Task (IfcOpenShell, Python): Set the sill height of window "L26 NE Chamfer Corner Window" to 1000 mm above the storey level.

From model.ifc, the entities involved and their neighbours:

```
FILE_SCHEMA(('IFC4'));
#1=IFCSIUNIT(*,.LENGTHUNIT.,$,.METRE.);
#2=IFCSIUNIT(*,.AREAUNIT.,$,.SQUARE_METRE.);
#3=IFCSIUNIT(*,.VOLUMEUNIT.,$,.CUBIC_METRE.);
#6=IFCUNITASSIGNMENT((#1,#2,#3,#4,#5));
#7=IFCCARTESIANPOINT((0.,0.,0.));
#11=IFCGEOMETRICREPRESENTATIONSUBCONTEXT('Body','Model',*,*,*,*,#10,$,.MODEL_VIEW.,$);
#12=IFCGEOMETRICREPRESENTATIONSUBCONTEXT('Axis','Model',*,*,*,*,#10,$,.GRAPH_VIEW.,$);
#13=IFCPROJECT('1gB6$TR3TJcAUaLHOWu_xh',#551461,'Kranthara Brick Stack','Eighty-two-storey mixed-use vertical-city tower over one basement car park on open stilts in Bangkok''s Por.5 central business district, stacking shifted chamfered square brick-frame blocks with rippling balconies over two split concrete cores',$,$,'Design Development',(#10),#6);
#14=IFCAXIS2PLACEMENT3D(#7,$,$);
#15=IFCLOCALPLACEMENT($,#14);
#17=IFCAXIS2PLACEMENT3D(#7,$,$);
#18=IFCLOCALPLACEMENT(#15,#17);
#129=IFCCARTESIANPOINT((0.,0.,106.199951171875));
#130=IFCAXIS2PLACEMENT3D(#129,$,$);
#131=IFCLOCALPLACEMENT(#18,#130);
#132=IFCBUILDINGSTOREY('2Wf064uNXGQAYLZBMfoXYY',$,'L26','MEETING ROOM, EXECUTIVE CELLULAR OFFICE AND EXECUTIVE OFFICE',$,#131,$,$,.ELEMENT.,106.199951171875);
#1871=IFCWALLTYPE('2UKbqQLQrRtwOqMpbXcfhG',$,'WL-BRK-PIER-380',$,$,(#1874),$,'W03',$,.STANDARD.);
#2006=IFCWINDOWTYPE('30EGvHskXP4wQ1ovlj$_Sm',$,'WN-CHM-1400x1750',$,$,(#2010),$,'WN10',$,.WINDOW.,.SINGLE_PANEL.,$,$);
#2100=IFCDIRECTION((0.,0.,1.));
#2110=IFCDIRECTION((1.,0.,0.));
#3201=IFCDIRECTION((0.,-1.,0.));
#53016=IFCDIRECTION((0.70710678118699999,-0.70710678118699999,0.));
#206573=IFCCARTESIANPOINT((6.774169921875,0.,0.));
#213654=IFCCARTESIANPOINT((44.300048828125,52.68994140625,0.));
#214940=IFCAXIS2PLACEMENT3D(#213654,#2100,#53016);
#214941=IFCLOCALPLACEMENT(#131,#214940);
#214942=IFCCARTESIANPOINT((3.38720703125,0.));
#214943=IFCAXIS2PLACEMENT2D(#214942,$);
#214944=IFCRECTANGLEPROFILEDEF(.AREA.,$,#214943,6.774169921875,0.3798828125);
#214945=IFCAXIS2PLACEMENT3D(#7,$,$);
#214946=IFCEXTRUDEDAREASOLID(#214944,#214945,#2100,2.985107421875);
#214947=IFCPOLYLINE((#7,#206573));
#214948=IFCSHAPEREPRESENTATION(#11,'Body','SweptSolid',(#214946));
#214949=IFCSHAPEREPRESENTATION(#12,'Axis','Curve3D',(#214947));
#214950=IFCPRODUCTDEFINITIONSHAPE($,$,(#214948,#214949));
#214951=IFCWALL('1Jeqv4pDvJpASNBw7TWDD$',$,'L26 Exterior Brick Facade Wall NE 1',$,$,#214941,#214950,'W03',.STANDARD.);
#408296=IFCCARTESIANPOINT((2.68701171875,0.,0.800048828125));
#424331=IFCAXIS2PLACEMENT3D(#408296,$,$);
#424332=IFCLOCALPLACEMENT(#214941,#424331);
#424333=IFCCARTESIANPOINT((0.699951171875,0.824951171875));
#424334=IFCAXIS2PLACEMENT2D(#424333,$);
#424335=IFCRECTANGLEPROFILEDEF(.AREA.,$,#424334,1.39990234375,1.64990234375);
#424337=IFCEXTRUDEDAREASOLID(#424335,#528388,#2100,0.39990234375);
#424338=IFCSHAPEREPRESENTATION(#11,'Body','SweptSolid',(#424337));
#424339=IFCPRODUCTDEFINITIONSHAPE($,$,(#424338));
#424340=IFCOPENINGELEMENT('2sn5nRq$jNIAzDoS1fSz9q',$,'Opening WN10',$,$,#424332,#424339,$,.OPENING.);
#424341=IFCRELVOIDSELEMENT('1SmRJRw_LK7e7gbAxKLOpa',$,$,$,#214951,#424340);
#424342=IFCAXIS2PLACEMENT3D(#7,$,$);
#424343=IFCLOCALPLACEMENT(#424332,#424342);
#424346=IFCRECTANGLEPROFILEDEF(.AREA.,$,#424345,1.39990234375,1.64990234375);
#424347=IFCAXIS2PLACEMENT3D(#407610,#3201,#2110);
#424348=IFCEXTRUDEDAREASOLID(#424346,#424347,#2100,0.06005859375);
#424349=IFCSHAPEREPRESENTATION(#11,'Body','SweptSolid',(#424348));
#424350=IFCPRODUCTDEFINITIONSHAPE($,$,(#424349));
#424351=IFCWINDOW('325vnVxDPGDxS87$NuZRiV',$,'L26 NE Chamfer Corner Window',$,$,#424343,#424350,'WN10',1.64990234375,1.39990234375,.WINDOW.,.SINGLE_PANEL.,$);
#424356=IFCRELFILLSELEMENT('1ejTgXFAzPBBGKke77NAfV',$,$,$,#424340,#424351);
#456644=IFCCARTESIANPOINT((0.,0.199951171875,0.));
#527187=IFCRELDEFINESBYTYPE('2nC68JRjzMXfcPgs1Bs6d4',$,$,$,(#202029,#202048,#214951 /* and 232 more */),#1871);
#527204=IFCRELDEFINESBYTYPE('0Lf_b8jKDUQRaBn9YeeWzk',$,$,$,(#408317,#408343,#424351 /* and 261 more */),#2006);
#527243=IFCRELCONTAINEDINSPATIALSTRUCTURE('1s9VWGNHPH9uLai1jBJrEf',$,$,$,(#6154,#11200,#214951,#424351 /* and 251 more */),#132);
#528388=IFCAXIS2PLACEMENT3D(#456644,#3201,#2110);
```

```python
import numpy as np
import ifcopenshell
import ifcopenshell.api.geometry
import ifcopenshell.geom
import ifcopenshell.util.element
import ifcopenshell.util.placement
import ifcopenshell.util.shape
import ifcopenshell.util.unit

model = ifcopenshell.open("model.ifc")
unit_scale = ifcopenshell.util.unit.calculate_unit_scale(model)

window = model.by_guid("325vnVxDPGDxS87$NuZRiV")
opening = window.FillsVoids[0].RelatingOpeningElement
storey = ifcopenshell.util.element.get_container(window, ifc_class="IfcBuildingStorey")
level = ifcopenshell.util.placement.get_local_placement(storey.ObjectPlacement)[2, 3]

# The opening's origin need not be at the sill, so measure its lowest point.
shape = ifcopenshell.geom.create_shape(ifcopenshell.geom.settings(), opening)
bottom = ifcopenshell.util.shape.get_shape_bottom_elevation(shape, shape.geometry) / unit_scale
dz = level + 1 / unit_scale - bottom

shift = np.array([0.0, 0.0, dz])
# The window is placed relative to its opening, so it follows when the opening moves.
matrix = ifcopenshell.util.placement.get_local_placement(opening.ObjectPlacement)
matrix[:3, 3] += shift
ifcopenshell.api.geometry.edit_object_placement(
    model, product=opening, matrix=matrix, is_si=False, should_transform_children=True
)

print(f"moved by {dz * unit_scale:+.3f} m")

model.write("model_updated.ifc")
```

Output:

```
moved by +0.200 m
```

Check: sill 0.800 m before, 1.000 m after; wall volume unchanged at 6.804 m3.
